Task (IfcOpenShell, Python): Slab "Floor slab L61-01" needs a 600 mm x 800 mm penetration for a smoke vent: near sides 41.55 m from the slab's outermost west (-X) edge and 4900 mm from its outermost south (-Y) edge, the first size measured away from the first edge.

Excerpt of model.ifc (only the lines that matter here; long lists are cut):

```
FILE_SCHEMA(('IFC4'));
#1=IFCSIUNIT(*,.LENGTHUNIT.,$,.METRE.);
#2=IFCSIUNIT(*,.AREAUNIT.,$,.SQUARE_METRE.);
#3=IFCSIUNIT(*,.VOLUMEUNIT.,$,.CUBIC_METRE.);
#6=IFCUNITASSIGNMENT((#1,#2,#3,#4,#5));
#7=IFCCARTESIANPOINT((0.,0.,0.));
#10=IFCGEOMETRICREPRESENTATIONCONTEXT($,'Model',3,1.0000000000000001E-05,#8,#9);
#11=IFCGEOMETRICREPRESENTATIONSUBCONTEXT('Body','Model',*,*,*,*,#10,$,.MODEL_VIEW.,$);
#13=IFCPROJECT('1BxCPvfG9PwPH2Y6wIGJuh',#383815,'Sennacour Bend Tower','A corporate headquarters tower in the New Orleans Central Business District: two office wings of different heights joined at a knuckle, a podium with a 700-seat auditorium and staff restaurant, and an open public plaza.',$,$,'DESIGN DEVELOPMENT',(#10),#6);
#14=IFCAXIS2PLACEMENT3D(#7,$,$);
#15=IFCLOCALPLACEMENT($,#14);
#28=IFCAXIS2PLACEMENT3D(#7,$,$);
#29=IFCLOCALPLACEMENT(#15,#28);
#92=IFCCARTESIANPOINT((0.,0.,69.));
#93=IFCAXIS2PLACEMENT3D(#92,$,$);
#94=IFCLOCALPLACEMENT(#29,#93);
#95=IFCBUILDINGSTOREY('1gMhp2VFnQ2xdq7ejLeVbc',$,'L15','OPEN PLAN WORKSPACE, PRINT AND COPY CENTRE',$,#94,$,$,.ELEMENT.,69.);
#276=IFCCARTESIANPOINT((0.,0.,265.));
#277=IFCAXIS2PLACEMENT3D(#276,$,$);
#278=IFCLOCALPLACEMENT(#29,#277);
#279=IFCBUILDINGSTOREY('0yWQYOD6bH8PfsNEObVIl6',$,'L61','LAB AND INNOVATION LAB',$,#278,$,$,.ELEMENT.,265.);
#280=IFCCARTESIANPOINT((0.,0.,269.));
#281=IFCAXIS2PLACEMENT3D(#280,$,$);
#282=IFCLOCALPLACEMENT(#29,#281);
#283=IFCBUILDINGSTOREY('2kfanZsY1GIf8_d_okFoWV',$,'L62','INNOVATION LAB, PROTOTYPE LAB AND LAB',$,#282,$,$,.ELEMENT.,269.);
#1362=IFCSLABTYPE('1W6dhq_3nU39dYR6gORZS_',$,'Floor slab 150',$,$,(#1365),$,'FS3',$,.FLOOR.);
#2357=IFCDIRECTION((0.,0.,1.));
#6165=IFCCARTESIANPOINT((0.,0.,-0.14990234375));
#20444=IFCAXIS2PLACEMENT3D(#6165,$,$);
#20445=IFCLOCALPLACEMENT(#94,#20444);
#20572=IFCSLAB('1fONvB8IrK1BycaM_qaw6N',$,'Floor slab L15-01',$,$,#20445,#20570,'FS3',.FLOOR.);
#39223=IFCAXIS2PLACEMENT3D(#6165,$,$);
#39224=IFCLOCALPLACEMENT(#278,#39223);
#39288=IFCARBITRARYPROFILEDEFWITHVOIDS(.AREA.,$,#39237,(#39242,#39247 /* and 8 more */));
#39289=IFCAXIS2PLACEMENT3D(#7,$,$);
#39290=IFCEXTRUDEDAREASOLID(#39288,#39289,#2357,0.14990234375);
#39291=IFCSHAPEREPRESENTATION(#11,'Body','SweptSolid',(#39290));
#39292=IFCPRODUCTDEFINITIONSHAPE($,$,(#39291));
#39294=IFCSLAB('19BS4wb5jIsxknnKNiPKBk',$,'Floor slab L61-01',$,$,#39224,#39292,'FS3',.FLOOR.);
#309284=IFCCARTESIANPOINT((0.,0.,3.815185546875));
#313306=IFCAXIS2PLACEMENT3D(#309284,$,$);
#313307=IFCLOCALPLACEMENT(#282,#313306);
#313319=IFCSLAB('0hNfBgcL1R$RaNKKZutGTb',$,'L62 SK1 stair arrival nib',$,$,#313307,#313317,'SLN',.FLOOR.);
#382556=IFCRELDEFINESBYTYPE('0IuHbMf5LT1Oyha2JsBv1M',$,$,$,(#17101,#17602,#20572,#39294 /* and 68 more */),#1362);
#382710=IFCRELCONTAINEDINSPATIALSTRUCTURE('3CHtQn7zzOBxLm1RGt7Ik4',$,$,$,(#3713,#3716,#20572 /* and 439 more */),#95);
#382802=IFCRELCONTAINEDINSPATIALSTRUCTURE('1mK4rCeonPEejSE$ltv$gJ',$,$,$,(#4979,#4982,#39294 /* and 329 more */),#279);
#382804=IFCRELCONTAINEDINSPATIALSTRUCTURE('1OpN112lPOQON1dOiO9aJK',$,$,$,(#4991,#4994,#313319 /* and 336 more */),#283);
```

```python
import numpy as np
import ifcopenshell
import ifcopenshell.api.feature
import ifcopenshell.api.geometry
import ifcopenshell.api.root
import ifcopenshell.geom
import ifcopenshell.util.placement
import ifcopenshell.util.representation
import ifcopenshell.util.shape
import ifcopenshell.util.unit

model = ifcopenshell.open("model.ifc")
unit_scale = ifcopenshell.util.unit.calculate_unit_scale(model)
settings = ifcopenshell.geom.settings()


def volume(element):
    """Net volume in cubic metres, openings subtracted."""
    shape = ifcopenshell.geom.create_shape(settings, element)
    return ifcopenshell.util.shape.get_volume(shape.geometry)


slab = model.by_guid("19BS4wb5jIsxknnKNiPKBk")
before = volume(slab)

# Extent in the slab's own axes, in metres. The edges named are its -X and -Y sides.
slab_shape = ifcopenshell.geom.create_shape(settings, slab)
vertices = ifcopenshell.util.shape.get_vertices(slab_shape.geometry)
x_min, y_min, bottom = vertices.min(axis=0)
top = vertices[:, 2].max()

opening = ifcopenshell.api.root.create_entity(model, ifc_class="IfcOpeningElement", name="Smoke vent opening", predefined_type="OPENING")
context = ifcopenshell.util.representation.get_context(model, "Model", "Body", "MODEL_VIEW")
width, depth = 0.6, 0.8
outline = [(0.0, 0.0), (width, 0.0), (width, depth), (0.0, depth), (0.0, 0.0)]
# Overshoot both faces by 50 mm so the cut is clean.
shape = ifcopenshell.api.geometry.add_slab_representation(
    model, context=context, depth=top - bottom + 0.1, polyline=outline
)
ifcopenshell.api.geometry.assign_representation(model, product=opening, representation=shape)

matrix = ifcopenshell.util.placement.get_local_placement(slab.ObjectPlacement)
matrix[:, 3] = matrix @ np.append(np.array([x_min + 41.55, y_min + 4.9, bottom - 0.05]) / unit_scale, 1.0)
ifcopenshell.api.geometry.edit_object_placement(model, product=opening, matrix=matrix, is_si=False)
ifcopenshell.api.feature.add_feature(model, feature=opening, element=slab)

after = volume(slab)

print(f"slab volume {before:.3f} -> {after:.3f} m3")

model.write("model-out.ifc")
```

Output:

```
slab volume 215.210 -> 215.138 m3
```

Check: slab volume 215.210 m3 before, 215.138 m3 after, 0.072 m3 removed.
